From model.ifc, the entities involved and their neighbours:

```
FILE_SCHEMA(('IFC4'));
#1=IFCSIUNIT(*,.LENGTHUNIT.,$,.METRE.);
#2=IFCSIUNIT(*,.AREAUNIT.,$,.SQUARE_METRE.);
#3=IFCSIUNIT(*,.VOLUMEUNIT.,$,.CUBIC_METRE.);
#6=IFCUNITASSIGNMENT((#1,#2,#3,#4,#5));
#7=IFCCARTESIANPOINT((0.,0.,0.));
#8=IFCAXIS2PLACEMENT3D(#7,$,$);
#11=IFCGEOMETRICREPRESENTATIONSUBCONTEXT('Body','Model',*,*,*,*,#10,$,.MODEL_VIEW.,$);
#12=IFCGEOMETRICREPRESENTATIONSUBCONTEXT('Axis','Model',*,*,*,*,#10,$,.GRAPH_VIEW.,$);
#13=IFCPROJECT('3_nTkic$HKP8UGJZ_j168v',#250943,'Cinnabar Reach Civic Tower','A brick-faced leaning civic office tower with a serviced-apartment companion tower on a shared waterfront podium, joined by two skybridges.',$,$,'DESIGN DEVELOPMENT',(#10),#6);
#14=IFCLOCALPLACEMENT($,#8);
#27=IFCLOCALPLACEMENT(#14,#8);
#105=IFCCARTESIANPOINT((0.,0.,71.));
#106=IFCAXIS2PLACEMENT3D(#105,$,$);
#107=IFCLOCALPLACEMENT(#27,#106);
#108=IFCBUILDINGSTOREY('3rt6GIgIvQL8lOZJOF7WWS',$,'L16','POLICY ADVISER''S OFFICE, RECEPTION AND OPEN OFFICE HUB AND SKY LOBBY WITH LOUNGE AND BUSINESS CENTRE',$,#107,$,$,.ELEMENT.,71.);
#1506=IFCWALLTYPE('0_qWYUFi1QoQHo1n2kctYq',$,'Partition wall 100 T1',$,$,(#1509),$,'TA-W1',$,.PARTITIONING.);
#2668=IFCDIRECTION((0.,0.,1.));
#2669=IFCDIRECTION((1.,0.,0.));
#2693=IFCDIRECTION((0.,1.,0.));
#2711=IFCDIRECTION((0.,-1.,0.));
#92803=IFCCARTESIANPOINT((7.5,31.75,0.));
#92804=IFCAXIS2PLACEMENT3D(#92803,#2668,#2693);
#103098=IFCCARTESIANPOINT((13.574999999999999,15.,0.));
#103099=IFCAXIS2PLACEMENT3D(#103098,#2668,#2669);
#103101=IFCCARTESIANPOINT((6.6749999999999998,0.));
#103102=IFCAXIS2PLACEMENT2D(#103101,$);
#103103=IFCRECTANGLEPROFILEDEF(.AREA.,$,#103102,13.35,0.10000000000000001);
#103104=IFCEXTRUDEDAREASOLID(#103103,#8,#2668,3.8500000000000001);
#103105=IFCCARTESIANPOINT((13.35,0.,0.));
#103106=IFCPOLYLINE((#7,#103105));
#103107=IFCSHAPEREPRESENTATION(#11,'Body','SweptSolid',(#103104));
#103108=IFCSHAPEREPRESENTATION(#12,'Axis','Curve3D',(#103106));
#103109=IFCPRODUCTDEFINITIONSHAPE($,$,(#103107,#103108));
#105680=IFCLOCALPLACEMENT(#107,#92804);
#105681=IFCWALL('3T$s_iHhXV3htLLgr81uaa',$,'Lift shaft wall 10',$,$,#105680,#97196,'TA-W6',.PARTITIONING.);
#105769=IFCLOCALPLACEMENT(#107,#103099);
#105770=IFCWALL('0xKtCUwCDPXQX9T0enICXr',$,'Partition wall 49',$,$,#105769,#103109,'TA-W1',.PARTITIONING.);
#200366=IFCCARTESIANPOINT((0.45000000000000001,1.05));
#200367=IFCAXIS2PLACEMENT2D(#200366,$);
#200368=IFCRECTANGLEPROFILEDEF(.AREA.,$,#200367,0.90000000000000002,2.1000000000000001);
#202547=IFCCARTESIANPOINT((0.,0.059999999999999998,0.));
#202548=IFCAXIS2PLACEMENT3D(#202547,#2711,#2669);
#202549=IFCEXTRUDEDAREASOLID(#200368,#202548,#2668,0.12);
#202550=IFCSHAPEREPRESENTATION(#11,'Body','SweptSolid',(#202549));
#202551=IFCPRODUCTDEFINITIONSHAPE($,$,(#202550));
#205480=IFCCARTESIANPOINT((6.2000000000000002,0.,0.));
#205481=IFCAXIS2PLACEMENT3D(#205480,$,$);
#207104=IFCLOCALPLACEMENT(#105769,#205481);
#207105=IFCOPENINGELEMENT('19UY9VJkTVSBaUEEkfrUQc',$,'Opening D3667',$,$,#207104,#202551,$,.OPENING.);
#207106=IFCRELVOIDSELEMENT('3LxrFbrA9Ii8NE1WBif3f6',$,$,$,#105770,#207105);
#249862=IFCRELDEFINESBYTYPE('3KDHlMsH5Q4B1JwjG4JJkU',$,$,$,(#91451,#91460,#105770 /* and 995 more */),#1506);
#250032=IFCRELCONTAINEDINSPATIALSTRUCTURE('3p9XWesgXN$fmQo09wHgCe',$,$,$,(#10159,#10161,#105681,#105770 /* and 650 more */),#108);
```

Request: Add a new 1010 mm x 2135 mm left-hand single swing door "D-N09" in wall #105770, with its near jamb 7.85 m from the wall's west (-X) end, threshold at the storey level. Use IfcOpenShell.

```python
import numpy as np
import ifcopenshell
import ifcopenshell.api.feature
import ifcopenshell.api.geometry
import ifcopenshell.api.root
import ifcopenshell.api.spatial
import ifcopenshell.geom
import ifcopenshell.util.element
import ifcopenshell.util.placement
import ifcopenshell.util.representation
import ifcopenshell.util.shape
import ifcopenshell.util.unit

model = ifcopenshell.open("model.ifc")
unit_scale = ifcopenshell.util.unit.calculate_unit_scale(model)
settings = ifcopenshell.geom.settings()


def volume(element):
    """Net volume in cubic metres, openings subtracted."""
    shape = ifcopenshell.geom.create_shape(settings, element)
    return ifcopenshell.util.shape.get_volume(shape.geometry)


wall = model.by_guid("0xKtCUwCDPXQX9T0enICXr")
storey = ifcopenshell.util.element.get_container(wall, ifc_class="IfcBuildingStorey")
context = ifcopenshell.util.representation.get_context(model, "Model", "Body", "MODEL_VIEW")
before = volume(wall)

width, height, from_end, sill = 1.01, 2.135, 7.85, 0.0  # metres

# The wall runs along its own X axis, and the end named is its -X end.
wall_shape = ifcopenshell.geom.create_shape(settings, wall)
x, y, z = ifcopenshell.util.shape.get_vertices(wall_shape.geometry).T
start = x.min() + from_end
face, thickness = float(y.min()), float(y.max() - y.min())
wall_matrix = ifcopenshell.util.placement.get_local_placement(wall.ObjectPlacement)
level = ifcopenshell.util.placement.get_local_placement(storey.ObjectPlacement)[2, 3]


def in_wall(x, y):
    """Placement at x, y metres in the wall's axes, at sill height."""
    matrix = wall_matrix.copy()
    matrix[:, 3] = wall_matrix @ np.array([x / unit_scale, y / unit_scale, 0.0, 1.0])
    matrix[2, 3] = level + sill / unit_scale
    return matrix


# Opening: a box that overshoots both wall faces by 50 mm.
opening = ifcopenshell.api.root.create_entity(model, ifc_class="IfcOpeningElement", predefined_type="OPENING")
box = ifcopenshell.api.geometry.add_wall_representation(
    model, context=context, length=width, height=height, thickness=thickness + 0.1
)
ifcopenshell.api.geometry.assign_representation(model, product=opening, representation=box)
ifcopenshell.api.geometry.edit_object_placement(model, product=opening, matrix=in_wall(start, face - 0.05), is_si=False)
ifcopenshell.api.feature.add_feature(model, feature=opening, element=wall)

door = ifcopenshell.api.root.create_entity(model, ifc_class="IfcDoor", name="D-N09", predefined_type="DOOR")
door.OverallWidth, door.OverallHeight = width / unit_scale, height / unit_scale
door.OperationType = "SINGLE_SWING_LEFT"
body = ifcopenshell.api.geometry.add_door_representation(
    model,
    context=context,
    overall_width=door.OverallWidth,
    overall_height=door.OverallHeight,
    operation_type="SINGLE_SWING_LEFT",
    lining_properties={"LiningDepth": thickness / unit_scale, "ThresholdDepth": thickness / unit_scale},
)
ifcopenshell.api.geometry.assign_representation(model, product=door, representation=body)
ifcopenshell.api.spatial.assign_container(model, products=[door], relating_structure=storey)
ifcopenshell.api.feature.add_filling(model, opening=opening, element=door)

# The lining spans the wall, so the door starts at the wall face.
ifcopenshell.api.geometry.edit_object_placement(model, product=door, matrix=in_wall(start, face), is_si=False)

after = volume(wall)

print(f"wall volume {before:.3f} -> {after:.3f} m3")

model.write("model_v2.ifc")
```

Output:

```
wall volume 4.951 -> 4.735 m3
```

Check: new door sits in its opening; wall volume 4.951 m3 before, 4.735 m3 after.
